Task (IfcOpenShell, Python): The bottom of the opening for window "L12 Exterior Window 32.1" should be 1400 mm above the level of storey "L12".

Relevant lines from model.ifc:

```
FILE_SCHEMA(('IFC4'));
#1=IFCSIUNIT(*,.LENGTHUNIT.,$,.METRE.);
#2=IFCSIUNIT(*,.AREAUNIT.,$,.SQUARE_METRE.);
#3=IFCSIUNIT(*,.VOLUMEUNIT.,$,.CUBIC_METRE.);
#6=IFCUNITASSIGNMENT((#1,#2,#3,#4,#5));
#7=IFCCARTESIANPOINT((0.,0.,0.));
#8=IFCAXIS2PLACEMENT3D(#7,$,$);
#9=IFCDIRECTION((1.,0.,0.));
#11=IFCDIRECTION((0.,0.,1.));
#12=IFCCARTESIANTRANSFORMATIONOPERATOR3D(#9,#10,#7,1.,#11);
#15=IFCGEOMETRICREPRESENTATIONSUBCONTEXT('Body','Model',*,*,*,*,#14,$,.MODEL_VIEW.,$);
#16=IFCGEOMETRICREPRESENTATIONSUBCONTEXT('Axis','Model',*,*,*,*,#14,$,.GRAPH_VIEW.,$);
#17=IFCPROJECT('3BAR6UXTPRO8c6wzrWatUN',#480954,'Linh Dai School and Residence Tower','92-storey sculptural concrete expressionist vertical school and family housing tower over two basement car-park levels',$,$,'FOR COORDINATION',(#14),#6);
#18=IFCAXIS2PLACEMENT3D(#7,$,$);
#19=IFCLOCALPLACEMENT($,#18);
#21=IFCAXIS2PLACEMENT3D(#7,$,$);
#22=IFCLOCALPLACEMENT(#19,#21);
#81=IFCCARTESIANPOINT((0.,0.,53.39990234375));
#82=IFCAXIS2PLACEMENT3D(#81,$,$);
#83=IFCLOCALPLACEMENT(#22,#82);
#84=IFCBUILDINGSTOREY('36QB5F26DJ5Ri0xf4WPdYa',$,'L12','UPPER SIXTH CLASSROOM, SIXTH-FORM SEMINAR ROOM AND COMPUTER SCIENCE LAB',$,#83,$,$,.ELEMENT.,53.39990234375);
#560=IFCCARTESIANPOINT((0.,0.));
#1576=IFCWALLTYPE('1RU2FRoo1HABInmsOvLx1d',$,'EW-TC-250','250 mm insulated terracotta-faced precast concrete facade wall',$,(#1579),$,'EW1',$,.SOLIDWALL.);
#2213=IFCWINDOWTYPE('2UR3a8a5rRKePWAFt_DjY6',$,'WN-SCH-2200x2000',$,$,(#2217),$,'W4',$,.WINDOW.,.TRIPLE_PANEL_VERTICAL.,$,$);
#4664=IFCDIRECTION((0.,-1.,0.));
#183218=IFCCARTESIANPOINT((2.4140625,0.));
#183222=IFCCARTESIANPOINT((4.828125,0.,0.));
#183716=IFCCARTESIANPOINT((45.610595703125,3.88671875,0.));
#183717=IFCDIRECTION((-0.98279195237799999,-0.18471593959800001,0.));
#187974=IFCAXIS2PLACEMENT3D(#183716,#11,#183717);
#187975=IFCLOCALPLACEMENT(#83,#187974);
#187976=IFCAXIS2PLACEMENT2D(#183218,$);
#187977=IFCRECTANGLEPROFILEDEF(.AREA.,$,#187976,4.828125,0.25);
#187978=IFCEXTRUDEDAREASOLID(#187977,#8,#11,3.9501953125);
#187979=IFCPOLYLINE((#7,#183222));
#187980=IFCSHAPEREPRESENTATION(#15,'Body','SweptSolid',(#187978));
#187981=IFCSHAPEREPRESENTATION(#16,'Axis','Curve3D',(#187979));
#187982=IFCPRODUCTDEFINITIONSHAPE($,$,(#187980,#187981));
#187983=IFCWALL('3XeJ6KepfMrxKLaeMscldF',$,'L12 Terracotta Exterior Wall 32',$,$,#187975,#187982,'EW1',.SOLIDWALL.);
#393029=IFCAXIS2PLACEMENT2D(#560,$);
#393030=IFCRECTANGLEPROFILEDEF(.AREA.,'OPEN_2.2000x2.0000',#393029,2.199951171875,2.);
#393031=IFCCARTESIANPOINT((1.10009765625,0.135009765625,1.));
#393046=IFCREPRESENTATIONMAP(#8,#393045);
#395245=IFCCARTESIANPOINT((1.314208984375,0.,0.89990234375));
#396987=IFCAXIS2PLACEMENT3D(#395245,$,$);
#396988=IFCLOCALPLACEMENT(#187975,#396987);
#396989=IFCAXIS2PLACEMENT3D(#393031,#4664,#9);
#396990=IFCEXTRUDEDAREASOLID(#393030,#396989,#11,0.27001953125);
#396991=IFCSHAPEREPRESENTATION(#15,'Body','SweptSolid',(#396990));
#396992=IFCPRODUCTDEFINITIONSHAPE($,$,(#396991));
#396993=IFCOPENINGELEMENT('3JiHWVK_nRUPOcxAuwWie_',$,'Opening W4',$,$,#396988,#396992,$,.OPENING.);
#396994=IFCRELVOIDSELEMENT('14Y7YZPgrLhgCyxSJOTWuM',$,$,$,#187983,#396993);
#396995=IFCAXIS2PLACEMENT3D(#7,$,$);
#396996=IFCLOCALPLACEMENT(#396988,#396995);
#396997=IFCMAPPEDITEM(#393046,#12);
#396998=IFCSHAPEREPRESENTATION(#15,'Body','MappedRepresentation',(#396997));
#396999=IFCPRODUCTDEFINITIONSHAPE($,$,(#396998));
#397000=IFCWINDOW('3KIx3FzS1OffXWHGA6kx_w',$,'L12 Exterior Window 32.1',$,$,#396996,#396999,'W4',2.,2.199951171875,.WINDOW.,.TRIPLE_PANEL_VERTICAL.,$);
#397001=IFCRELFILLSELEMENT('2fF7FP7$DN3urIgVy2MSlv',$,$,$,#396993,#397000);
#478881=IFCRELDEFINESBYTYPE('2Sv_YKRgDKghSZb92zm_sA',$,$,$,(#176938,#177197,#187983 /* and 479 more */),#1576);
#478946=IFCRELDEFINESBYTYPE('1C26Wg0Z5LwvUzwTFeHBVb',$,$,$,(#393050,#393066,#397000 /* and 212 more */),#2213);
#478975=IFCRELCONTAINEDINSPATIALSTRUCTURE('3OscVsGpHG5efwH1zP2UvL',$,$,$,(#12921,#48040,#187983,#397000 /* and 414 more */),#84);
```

```python
import numpy as np
import ifcopenshell
import ifcopenshell.api.geometry
import ifcopenshell.geom
import ifcopenshell.util.element
import ifcopenshell.util.placement
import ifcopenshell.util.shape
import ifcopenshell.util.unit

model = ifcopenshell.open("model.ifc")
unit_scale = ifcopenshell.util.unit.calculate_unit_scale(model)

window = model.by_guid("3KIx3FzS1OffXWHGA6kx_w")
opening = window.FillsVoids[0].RelatingOpeningElement
storey = ifcopenshell.util.element.get_container(window, ifc_class="IfcBuildingStorey")
level = ifcopenshell.util.placement.get_local_placement(storey.ObjectPlacement)[2, 3]

# The opening's origin need not be at the sill, so measure its lowest point.
shape = ifcopenshell.geom.create_shape(ifcopenshell.geom.settings(), opening)
bottom = ifcopenshell.util.shape.get_shape_bottom_elevation(shape, shape.geometry) / unit_scale
dz = level + 1.4 - bottom

shift = np.array([0.0, 0.0, dz])
# The window is placed relative to its opening, so it follows when the opening moves.
matrix = ifcopenshell.util.placement.get_local_placement(opening.ObjectPlacement)
matrix[:3, 3] += shift
ifcopenshell.api.geometry.edit_object_placement(
    model, product=opening, matrix=matrix, is_si=False, should_transform_children=True
)

print(f"moved by {dz * unit_scale:+.3f} m")

model.write("model_rev.ifc")
```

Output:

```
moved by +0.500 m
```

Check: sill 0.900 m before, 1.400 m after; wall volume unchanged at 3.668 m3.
